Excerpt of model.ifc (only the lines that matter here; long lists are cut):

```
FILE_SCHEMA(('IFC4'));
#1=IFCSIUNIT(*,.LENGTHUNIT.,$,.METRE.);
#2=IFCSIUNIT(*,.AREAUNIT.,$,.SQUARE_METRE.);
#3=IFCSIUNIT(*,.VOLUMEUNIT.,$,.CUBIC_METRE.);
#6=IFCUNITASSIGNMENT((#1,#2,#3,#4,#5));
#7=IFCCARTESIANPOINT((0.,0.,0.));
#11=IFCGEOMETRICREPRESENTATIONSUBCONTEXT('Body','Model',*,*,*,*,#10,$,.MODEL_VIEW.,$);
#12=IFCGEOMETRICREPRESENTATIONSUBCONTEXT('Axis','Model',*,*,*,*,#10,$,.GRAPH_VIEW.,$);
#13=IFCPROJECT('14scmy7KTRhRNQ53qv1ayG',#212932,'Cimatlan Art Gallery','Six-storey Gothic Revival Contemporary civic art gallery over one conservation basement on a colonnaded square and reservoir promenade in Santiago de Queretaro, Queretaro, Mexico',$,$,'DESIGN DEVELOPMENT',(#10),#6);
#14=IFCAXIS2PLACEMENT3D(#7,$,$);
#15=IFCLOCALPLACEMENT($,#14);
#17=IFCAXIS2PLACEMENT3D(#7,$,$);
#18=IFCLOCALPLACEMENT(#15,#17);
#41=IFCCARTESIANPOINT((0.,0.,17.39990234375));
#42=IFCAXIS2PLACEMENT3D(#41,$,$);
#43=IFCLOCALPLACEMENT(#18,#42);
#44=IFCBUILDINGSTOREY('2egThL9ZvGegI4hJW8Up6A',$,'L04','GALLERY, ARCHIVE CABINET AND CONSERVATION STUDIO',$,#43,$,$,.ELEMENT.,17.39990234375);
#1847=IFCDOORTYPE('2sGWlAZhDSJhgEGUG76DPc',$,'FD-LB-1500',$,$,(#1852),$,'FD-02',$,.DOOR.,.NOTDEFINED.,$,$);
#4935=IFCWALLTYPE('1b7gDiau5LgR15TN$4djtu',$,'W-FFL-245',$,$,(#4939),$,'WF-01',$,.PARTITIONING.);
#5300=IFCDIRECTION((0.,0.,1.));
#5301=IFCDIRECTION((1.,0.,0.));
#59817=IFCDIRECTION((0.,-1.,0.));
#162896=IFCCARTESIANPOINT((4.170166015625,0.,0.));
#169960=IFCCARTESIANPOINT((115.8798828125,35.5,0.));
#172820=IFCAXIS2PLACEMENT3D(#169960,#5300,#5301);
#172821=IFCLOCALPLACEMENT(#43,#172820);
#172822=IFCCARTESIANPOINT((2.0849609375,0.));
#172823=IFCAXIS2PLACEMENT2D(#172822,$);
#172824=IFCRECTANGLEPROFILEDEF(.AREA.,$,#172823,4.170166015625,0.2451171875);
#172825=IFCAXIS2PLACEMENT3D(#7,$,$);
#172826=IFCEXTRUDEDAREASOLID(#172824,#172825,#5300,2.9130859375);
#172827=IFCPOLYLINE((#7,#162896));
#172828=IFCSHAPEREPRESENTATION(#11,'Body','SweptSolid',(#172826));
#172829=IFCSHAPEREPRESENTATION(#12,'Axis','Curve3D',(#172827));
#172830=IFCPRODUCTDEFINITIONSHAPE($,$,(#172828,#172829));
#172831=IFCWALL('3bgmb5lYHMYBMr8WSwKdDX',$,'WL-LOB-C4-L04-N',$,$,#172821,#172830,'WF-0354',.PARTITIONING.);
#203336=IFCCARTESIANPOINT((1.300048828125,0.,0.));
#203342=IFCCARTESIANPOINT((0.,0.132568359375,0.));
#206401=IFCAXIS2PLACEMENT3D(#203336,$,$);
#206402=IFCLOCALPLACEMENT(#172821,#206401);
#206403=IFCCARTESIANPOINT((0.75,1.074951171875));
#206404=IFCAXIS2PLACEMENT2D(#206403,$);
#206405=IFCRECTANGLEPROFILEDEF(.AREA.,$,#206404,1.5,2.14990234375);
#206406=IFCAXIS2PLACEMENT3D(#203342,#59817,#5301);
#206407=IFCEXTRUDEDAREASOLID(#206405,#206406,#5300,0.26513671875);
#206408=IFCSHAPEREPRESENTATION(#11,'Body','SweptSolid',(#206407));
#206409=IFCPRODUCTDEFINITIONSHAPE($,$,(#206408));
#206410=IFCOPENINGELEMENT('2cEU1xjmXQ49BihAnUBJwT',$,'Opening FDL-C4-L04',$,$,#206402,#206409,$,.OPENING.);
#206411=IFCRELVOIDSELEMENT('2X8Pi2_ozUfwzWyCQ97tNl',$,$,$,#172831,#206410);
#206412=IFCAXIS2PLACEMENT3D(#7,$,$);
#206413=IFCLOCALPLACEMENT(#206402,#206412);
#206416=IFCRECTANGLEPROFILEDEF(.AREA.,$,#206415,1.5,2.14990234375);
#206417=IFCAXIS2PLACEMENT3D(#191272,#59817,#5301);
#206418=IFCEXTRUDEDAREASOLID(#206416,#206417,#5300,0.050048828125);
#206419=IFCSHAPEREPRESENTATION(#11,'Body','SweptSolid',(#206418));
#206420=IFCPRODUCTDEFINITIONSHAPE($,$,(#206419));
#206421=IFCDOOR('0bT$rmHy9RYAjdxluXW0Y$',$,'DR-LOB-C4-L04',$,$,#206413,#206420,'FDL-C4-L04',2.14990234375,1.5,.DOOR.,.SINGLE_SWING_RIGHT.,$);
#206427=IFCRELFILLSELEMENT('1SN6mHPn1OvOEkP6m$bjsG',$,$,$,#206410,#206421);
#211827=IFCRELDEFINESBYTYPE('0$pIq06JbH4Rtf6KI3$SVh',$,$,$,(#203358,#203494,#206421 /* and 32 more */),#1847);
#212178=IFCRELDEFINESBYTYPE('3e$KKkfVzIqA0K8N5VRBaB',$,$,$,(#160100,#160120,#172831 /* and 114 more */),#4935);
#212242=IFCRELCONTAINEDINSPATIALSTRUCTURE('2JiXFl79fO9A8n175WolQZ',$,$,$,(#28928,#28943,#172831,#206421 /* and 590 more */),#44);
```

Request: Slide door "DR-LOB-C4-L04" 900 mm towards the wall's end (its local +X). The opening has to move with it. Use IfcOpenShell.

```python
import ifcopenshell
import ifcopenshell.api.geometry
import ifcopenshell.util.placement
import ifcopenshell.util.unit

model = ifcopenshell.open("model.ifc")
unit_scale = ifcopenshell.util.unit.calculate_unit_scale(model)

door = model.by_guid("0bT$rmHy9RYAjdxluXW0Y$")
opening = door.FillsVoids[0].RelatingOpeningElement
wall = opening.VoidsElements[0].RelatingBuildingElement

wall_matrix = ifcopenshell.util.placement.get_local_placement(wall.ObjectPlacement)
shift = wall_matrix[:3, 0] * 0.9 / unit_scale
before = ifcopenshell.util.placement.get_local_placement(door.ObjectPlacement)[:3, 3].copy()

# The door is placed relative to its opening, so it follows when the opening moves.
matrix = ifcopenshell.util.placement.get_local_placement(opening.ObjectPlacement)
matrix[:3, 3] += shift
ifcopenshell.api.geometry.edit_object_placement(
    model, product=opening, matrix=matrix, is_si=False, should_transform_children=True
)

after = ifcopenshell.util.placement.get_local_placement(door.ObjectPlacement)[:3, 3]
print("door moved by", (after - before).round(3) + 0.0)

model.write("model_v2.ifc")
```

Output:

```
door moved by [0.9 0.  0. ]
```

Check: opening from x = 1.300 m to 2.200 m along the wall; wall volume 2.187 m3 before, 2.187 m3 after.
